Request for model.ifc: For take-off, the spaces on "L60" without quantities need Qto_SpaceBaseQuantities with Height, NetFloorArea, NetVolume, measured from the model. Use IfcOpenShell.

First a look at what the model holds.

```python
import ifcopenshell
import ifcopenshell.util.element
import ifcopenshell.util.unit

model = ifcopenshell.open("model.ifc")
print(model.schema)
for unit_type in ("LENGTHUNIT", "AREAUNIT", "VOLUMEUNIT"):
    print(unit_type, ifcopenshell.util.unit.calculate_unit_scale(model, unit_type))
storey = next(s for s in model.by_type("IfcBuildingStorey") if s.Name == "L60")
spaces = [e for e in ifcopenshell.util.element.get_decomposition(storey) if e.is_a("IfcSpace")]
for e in sorted(spaces, key=lambda e: e.id()):
    print(e.id(), e.is_a(), e.Name, list(ifcopenshell.util.element.get_psets(e, qtos_only=True)), sep=" | ")
```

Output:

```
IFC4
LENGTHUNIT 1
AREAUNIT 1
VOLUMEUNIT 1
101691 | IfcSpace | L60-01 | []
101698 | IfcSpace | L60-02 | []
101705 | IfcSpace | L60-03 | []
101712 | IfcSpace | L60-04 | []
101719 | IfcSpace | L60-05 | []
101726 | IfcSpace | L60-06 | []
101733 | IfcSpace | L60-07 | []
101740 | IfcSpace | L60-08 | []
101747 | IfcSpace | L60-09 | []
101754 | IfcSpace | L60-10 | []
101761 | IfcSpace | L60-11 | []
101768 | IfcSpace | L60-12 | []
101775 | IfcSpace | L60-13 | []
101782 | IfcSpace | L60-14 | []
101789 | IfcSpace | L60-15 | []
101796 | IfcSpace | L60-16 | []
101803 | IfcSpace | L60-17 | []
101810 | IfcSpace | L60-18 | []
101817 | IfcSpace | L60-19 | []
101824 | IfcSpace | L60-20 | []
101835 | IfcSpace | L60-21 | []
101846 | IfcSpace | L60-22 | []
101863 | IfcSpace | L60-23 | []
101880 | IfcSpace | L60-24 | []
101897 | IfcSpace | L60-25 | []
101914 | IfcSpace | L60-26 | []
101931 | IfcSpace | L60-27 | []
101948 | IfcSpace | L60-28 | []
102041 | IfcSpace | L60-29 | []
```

```python
import ifcopenshell
import ifcopenshell.api.pset
import ifcopenshell.geom
import ifcopenshell.util.element
import ifcopenshell.util.shape
import ifcopenshell.util.unit

model = ifcopenshell.open("model.ifc")
unit_scale = ifcopenshell.util.unit.calculate_unit_scale(model)
area_scale = ifcopenshell.util.unit.calculate_unit_scale(model, "AREAUNIT")
volume_scale = ifcopenshell.util.unit.calculate_unit_scale(model, "VOLUMEUNIT")
settings = ifcopenshell.geom.settings()

storey = next(s for s in model.by_type("IfcBuildingStorey") if s.Name == "L60")
spaces = [e for e in ifcopenshell.util.element.get_decomposition(storey) if e.is_a("IfcSpace")]

for e in sorted(spaces, key=lambda e: e.id()):
    if ifcopenshell.util.element.get_psets(e, qtos_only=True, should_inherit=False):
        continue
    # Geometry comes back in metres, in the element's own axes.
    shape = ifcopenshell.geom.create_shape(settings, e)
    values = {
        "Height": ifcopenshell.util.shape.get_z(shape.geometry) / unit_scale,
        "NetFloorArea": ifcopenshell.util.shape.get_footprint_area(shape.geometry) / area_scale,
        "NetVolume": ifcopenshell.util.shape.get_volume(shape.geometry) / volume_scale,
    }
    qto = ifcopenshell.api.pset.add_qto(model, product=e, name="Qto_SpaceBaseQuantities")
    ifcopenshell.api.pset.edit_qto(model, qto=qto, properties=values)
    print(e.id(), {k: round(v, 3) for k, v in values.items()})

model.write("model_rev.ifc")
```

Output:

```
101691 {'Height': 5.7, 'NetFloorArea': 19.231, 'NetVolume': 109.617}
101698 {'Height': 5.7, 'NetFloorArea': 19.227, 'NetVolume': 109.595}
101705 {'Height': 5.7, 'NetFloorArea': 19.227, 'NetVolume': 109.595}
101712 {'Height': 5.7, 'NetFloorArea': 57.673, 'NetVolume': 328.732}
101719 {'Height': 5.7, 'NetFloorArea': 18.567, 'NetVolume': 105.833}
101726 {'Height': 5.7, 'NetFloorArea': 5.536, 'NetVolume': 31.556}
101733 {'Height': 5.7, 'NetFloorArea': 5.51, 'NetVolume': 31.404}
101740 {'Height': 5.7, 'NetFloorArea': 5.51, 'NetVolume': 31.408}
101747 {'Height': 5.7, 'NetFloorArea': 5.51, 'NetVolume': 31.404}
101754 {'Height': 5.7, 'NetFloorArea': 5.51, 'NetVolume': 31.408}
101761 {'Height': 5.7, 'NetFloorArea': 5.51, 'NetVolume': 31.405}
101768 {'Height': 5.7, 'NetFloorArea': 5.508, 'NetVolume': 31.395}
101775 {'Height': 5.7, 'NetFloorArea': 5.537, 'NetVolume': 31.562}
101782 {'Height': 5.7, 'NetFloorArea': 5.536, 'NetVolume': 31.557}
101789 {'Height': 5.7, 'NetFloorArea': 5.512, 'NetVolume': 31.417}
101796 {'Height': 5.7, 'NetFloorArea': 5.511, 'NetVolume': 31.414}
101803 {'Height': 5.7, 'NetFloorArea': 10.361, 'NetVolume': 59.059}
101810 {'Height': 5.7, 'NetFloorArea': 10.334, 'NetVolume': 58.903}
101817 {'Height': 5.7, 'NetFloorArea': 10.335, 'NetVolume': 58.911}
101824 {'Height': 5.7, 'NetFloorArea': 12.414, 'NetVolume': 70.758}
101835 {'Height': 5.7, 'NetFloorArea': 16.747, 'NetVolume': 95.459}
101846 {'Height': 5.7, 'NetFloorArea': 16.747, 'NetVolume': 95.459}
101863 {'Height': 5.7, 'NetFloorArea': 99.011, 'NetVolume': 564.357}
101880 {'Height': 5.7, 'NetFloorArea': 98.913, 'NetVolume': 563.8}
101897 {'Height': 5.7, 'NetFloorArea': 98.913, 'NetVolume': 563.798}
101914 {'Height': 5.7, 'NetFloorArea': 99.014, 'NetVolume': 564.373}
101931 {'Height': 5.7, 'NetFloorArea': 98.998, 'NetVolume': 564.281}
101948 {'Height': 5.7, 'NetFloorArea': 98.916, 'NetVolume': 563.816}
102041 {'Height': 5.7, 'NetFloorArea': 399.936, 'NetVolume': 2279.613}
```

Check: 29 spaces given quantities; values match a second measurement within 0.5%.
